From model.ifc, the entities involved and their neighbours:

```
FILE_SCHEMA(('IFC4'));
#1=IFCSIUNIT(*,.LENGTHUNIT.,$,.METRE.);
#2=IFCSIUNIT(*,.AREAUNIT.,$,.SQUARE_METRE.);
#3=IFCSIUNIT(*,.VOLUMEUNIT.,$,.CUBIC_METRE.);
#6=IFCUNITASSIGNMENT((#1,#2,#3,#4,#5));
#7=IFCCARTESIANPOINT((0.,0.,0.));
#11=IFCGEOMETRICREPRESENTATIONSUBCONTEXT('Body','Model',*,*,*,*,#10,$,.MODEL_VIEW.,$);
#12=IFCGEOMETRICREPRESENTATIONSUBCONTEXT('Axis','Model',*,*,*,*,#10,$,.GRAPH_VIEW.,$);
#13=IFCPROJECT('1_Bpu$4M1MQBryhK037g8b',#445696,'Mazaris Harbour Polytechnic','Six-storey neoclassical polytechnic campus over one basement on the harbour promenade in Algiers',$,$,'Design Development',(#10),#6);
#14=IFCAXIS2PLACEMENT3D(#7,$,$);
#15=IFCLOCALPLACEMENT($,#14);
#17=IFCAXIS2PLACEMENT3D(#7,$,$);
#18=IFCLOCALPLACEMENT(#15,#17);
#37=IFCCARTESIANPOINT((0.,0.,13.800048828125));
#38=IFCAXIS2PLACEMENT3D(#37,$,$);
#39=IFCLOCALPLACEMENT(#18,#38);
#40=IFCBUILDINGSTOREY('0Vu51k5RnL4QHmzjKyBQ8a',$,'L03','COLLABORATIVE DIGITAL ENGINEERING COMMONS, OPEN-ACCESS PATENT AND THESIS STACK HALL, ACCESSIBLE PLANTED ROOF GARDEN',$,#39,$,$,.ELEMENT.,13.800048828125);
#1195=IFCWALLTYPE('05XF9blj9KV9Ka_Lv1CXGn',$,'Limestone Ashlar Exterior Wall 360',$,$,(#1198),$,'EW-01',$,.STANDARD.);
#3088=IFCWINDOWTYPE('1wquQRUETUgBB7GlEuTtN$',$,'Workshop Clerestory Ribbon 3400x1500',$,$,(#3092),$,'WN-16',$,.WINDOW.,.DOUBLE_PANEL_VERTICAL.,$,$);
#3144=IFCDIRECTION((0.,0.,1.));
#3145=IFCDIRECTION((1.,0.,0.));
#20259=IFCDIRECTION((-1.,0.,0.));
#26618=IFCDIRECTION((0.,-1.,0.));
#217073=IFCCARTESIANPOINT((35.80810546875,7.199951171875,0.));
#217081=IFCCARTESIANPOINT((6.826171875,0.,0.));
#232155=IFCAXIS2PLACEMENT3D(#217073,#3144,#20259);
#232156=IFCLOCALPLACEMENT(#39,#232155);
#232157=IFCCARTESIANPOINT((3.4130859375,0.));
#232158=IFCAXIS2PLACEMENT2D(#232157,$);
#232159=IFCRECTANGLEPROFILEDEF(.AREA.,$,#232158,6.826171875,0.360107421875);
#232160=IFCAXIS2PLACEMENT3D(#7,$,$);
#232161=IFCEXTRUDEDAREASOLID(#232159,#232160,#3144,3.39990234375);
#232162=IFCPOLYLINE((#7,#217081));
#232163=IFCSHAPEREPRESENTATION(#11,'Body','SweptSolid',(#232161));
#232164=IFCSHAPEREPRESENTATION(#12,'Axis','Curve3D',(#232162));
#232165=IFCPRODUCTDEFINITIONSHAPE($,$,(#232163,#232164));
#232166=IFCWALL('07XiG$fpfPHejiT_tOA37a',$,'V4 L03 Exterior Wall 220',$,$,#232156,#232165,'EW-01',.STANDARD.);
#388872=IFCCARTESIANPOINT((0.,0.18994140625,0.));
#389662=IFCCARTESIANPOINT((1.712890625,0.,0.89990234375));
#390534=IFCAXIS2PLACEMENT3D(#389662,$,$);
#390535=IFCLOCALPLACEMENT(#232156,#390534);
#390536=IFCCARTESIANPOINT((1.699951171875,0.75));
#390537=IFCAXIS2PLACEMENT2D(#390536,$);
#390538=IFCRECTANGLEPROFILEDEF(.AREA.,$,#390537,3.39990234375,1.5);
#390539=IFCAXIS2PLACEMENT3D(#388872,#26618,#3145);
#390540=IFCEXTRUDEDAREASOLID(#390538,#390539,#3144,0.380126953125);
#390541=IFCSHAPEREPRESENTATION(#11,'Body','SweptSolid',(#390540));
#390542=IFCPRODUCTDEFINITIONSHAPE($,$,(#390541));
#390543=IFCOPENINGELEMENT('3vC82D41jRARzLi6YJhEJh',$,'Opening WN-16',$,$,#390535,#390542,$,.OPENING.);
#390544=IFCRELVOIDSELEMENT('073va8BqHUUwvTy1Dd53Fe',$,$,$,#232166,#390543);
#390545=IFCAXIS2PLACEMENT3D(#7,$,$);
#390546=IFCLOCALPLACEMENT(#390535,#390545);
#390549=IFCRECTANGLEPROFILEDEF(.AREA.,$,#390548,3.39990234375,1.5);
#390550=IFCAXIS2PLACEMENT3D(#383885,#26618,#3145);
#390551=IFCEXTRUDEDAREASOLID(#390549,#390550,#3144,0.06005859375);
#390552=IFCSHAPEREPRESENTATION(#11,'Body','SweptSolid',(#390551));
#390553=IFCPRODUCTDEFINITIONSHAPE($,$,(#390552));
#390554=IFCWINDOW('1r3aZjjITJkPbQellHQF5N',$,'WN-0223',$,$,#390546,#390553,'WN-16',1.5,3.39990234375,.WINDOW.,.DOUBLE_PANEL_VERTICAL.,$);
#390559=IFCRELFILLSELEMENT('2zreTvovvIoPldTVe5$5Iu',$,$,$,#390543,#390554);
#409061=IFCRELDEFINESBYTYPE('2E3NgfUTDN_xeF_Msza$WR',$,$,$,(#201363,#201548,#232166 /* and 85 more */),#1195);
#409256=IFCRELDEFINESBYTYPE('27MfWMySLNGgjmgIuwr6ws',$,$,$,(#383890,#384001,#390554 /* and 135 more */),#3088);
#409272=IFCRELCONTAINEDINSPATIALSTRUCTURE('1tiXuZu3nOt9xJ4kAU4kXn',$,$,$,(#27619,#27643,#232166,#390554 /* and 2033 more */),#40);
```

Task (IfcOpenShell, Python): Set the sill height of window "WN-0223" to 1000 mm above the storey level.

```python
import numpy as np
import ifcopenshell
import ifcopenshell.api.geometry
import ifcopenshell.geom
import ifcopenshell.util.element
import ifcopenshell.util.placement
import ifcopenshell.util.shape
import ifcopenshell.util.unit

model = ifcopenshell.open("model.ifc")
unit_scale = ifcopenshell.util.unit.calculate_unit_scale(model)

window = model.by_guid("1r3aZjjITJkPbQellHQF5N")
opening = window.FillsVoids[0].RelatingOpeningElement
storey = ifcopenshell.util.element.get_container(window, ifc_class="IfcBuildingStorey")
level = ifcopenshell.util.placement.get_local_placement(storey.ObjectPlacement)[2, 3]

# The opening's origin need not be at the sill, so measure its lowest point.
shape = ifcopenshell.geom.create_shape(ifcopenshell.geom.settings(), opening)
bottom = ifcopenshell.util.shape.get_shape_bottom_elevation(shape, shape.geometry) / unit_scale
dz = level + 1 / unit_scale - bottom

shift = np.array([0.0, 0.0, dz])
# The window is placed relative to its opening, so it follows when the opening moves.
matrix = ifcopenshell.util.placement.get_local_placement(opening.ObjectPlacement)
matrix[:3, 3] += shift
ifcopenshell.api.geometry.edit_object_placement(
    model, product=opening, matrix=matrix, is_si=False, should_transform_children=True
)

print(f"moved by {dz * unit_scale:+.3f} m")

model.write("model_rev.ifc")
```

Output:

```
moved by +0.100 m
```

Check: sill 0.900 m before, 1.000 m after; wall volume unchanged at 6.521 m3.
